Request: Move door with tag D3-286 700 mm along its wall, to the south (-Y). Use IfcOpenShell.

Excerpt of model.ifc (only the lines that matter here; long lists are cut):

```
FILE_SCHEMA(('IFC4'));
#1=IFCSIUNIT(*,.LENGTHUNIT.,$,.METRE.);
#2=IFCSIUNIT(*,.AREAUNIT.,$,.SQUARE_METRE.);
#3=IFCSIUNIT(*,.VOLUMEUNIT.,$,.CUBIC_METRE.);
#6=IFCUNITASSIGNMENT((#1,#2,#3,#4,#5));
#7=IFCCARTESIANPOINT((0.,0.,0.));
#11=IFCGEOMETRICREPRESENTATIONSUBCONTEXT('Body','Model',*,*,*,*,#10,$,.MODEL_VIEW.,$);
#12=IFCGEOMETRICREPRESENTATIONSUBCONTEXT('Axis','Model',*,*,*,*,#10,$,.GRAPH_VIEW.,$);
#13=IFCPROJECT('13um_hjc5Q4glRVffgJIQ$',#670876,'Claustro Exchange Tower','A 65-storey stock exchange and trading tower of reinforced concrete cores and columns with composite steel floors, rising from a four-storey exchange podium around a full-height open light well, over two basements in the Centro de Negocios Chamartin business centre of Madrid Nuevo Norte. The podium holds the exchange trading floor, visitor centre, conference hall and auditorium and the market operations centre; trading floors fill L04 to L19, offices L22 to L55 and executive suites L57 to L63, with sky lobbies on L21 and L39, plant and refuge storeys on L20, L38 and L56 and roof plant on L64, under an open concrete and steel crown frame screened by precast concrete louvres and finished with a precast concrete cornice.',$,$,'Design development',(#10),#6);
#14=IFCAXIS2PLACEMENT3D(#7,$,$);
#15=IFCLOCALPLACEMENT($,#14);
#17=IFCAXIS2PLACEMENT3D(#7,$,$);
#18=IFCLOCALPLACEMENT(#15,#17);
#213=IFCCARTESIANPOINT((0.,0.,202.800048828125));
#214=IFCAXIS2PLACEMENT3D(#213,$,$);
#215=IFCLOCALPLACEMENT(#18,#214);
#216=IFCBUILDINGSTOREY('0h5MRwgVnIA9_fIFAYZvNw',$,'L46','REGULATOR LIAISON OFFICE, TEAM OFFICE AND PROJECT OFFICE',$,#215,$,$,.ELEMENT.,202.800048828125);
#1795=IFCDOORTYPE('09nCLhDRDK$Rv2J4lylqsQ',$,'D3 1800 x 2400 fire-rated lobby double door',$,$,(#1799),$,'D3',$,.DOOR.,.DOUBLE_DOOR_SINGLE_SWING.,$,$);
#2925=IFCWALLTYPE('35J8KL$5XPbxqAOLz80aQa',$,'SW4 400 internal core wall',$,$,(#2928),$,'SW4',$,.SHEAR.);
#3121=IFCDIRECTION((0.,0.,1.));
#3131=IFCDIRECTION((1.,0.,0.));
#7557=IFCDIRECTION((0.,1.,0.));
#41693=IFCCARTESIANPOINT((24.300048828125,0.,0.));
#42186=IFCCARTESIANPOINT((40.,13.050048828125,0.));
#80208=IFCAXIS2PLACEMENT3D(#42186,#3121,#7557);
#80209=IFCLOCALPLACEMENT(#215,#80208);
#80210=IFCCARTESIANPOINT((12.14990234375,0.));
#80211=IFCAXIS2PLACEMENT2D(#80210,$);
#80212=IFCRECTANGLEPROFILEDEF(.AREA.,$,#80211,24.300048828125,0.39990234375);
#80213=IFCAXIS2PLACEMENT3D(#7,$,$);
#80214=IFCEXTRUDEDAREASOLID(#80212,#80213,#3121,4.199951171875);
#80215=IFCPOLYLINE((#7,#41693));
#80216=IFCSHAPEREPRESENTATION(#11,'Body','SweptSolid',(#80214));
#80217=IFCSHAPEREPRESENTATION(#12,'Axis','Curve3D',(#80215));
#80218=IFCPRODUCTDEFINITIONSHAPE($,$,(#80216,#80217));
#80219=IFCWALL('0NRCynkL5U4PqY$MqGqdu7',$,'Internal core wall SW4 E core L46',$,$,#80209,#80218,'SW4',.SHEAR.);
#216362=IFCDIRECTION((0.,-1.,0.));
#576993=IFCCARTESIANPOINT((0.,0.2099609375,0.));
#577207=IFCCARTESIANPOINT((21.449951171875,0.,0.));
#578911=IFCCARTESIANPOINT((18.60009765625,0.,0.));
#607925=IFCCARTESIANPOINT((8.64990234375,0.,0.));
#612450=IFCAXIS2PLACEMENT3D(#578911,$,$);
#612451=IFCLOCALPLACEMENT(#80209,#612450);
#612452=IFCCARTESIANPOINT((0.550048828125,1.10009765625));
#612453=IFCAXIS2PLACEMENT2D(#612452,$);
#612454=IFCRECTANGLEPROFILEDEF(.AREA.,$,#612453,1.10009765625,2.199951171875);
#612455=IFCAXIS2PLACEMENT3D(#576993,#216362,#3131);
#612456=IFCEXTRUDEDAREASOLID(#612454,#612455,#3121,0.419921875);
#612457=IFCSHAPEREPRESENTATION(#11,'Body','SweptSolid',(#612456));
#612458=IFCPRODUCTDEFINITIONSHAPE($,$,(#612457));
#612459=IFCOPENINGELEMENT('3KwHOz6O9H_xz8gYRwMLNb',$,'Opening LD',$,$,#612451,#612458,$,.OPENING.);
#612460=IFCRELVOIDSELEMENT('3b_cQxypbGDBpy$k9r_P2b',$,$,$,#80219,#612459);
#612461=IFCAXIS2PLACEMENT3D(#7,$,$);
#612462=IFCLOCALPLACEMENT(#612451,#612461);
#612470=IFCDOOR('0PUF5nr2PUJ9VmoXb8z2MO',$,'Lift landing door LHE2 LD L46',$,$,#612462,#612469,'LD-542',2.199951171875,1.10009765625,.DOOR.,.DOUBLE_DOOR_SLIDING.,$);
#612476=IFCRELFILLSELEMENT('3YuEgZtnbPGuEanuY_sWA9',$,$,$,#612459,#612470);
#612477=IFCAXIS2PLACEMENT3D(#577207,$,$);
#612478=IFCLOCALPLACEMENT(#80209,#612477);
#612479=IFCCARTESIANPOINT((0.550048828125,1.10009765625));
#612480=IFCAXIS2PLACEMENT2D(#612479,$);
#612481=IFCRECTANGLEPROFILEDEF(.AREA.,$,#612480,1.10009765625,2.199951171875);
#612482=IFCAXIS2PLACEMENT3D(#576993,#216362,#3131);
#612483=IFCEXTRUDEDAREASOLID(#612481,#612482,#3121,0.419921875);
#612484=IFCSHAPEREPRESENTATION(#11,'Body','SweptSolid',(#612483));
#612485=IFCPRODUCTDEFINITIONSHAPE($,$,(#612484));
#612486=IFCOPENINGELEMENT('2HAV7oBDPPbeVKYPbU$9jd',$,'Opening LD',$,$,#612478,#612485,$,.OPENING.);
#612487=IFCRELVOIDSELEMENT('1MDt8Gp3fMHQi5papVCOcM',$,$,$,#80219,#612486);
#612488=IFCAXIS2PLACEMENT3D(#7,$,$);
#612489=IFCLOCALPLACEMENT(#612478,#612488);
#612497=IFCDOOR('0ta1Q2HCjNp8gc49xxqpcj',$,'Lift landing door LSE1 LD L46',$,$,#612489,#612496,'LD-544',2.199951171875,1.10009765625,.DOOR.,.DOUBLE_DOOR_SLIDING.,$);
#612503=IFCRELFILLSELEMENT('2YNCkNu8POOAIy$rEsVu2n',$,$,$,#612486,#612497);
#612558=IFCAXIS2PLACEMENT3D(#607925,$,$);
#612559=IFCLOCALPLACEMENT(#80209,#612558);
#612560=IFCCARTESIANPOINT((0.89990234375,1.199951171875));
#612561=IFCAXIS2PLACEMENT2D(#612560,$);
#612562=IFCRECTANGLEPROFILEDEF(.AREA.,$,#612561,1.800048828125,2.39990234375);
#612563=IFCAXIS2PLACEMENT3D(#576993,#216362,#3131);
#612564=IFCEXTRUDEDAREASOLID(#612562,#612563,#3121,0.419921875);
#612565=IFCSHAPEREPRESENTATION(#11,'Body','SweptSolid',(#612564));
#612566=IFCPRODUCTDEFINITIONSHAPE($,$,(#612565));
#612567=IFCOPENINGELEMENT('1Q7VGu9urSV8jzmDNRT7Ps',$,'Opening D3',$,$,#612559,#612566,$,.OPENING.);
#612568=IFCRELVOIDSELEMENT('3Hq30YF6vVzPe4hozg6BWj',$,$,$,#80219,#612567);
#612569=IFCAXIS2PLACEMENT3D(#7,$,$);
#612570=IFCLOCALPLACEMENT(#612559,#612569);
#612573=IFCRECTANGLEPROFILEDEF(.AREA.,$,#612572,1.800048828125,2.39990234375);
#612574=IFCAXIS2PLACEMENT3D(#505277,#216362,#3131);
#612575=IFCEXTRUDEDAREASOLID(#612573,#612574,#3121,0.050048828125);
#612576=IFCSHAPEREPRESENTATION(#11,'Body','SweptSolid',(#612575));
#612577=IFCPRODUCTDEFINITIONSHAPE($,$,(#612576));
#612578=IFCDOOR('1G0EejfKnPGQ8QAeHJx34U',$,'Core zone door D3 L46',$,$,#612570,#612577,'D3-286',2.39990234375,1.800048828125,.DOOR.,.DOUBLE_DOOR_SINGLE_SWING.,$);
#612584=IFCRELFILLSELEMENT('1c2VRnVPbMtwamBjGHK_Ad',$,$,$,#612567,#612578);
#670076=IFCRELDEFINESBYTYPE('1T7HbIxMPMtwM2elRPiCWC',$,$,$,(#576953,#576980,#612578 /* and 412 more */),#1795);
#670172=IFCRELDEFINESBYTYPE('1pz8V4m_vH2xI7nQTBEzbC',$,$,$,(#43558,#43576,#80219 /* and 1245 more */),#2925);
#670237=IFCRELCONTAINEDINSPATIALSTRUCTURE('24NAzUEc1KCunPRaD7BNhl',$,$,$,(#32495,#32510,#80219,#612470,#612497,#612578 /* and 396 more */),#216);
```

```python
import ifcopenshell
import ifcopenshell.api.geometry
import ifcopenshell.util.placement
import ifcopenshell.util.unit

model = ifcopenshell.open("model.ifc")
unit_scale = ifcopenshell.util.unit.calculate_unit_scale(model)

door = model.by_guid("1G0EejfKnPGQ8QAeHJx34U")
opening = door.FillsVoids[0].RelatingOpeningElement
wall = opening.VoidsElements[0].RelatingBuildingElement

wall_matrix = ifcopenshell.util.placement.get_local_placement(wall.ObjectPlacement)
shift = wall_matrix[:3, 0] * -0.7 / unit_scale
before = ifcopenshell.util.placement.get_local_placement(door.ObjectPlacement)[:3, 3].copy()

# The door is placed relative to its opening, so it follows when the opening moves.
matrix = ifcopenshell.util.placement.get_local_placement(opening.ObjectPlacement)
matrix[:3, 3] += shift
ifcopenshell.api.geometry.edit_object_placement(
    model, product=opening, matrix=matrix, is_si=False, should_transform_children=True
)

after = ifcopenshell.util.placement.get_local_placement(door.ObjectPlacement)[:3, 3]
print("door moved by", (after - before).round(3) + 0.0)

model.write("model_rev.ifc")
```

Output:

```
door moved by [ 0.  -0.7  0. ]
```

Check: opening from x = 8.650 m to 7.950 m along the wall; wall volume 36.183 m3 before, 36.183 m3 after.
